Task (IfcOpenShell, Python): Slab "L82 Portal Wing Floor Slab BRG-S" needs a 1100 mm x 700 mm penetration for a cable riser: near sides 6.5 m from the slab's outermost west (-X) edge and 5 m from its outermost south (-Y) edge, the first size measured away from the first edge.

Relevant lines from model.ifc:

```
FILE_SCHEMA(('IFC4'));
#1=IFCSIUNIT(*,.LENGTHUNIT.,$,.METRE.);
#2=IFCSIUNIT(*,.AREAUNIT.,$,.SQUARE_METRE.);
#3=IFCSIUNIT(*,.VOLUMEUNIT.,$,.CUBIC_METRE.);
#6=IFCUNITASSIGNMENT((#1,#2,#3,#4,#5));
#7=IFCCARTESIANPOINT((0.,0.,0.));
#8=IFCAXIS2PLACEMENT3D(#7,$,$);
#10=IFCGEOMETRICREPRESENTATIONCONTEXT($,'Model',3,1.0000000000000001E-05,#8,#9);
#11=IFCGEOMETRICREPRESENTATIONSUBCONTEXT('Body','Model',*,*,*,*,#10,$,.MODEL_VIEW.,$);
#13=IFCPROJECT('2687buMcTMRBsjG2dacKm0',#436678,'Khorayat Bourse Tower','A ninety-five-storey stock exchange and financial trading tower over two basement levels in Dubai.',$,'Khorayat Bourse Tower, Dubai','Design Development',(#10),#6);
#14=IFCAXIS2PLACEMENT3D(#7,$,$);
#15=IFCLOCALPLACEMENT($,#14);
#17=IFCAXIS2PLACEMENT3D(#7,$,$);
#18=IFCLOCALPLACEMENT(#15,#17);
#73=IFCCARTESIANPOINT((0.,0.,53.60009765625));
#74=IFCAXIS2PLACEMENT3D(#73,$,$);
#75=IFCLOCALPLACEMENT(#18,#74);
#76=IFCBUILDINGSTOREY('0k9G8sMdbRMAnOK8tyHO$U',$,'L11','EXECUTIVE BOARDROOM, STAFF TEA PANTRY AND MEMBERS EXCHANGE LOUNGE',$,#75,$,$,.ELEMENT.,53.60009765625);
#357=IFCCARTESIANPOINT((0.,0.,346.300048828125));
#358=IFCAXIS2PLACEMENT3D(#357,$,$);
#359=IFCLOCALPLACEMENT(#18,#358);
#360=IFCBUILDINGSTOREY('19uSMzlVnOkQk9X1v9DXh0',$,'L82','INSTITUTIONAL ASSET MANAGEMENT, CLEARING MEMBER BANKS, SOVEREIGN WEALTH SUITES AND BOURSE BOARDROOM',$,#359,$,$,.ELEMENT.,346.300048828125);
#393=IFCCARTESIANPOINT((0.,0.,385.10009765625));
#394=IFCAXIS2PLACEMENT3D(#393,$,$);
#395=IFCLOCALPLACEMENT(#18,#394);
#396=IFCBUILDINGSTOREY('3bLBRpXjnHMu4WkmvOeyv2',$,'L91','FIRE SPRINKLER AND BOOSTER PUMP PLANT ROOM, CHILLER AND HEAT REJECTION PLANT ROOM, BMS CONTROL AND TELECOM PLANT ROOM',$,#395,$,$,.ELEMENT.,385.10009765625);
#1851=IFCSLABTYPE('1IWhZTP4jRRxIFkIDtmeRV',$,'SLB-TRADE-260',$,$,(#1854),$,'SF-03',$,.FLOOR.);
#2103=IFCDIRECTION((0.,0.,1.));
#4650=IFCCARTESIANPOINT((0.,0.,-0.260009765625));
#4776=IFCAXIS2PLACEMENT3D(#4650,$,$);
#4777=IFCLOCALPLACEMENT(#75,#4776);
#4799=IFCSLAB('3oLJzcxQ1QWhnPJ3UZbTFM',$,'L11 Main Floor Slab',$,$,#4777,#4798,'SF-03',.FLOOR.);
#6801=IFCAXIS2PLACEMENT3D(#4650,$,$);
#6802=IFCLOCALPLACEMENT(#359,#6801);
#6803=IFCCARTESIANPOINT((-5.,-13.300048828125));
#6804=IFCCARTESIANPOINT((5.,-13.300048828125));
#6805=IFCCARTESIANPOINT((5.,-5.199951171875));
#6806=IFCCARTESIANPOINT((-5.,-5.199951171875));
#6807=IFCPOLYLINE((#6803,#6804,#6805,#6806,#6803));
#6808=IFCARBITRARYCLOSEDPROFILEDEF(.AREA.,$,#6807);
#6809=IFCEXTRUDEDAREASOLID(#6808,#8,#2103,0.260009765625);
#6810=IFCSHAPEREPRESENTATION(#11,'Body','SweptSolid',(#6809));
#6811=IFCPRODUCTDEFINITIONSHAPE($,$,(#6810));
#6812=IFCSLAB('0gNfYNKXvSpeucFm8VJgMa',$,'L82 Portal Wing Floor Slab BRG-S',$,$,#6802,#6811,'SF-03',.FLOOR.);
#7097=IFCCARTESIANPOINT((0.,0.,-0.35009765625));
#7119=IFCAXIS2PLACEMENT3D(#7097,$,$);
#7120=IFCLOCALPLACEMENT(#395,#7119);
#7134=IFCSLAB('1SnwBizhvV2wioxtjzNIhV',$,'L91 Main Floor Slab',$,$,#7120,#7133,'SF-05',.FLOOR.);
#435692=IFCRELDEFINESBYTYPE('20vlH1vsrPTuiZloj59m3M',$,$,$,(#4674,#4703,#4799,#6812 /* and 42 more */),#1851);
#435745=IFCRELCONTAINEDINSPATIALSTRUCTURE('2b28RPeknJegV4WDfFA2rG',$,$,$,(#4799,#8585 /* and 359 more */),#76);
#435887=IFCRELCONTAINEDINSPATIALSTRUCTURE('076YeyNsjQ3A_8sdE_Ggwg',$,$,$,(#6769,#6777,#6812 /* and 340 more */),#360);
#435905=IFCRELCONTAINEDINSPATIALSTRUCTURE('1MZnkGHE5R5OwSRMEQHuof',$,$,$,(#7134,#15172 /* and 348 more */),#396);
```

```python
import numpy as np
import ifcopenshell
import ifcopenshell.api.feature
import ifcopenshell.api.geometry
import ifcopenshell.api.root
import ifcopenshell.geom
import ifcopenshell.util.placement
import ifcopenshell.util.representation
import ifcopenshell.util.shape
import ifcopenshell.util.unit

model = ifcopenshell.open("model.ifc")
unit_scale = ifcopenshell.util.unit.calculate_unit_scale(model)
settings = ifcopenshell.geom.settings()


def volume(element):
    """Net volume in cubic metres, openings subtracted."""
    shape = ifcopenshell.geom.create_shape(settings, element)
    return ifcopenshell.util.shape.get_volume(shape.geometry)


slab = model.by_id(6812)
before = volume(slab)

# Extent in the slab's own axes, in metres. The edges named are its -X and -Y sides.
slab_shape = ifcopenshell.geom.create_shape(settings, slab)
vertices = ifcopenshell.util.shape.get_vertices(slab_shape.geometry)
x_min, y_min, bottom = vertices.min(axis=0)
top = vertices[:, 2].max()

opening = ifcopenshell.api.root.create_entity(model, ifc_class="IfcOpeningElement", name="Cable riser opening", predefined_type="OPENING")
context = ifcopenshell.util.representation.get_context(model, "Model", "Body", "MODEL_VIEW")
width, depth = 1.1, 0.7
outline = [(0.0, 0.0), (width, 0.0), (width, depth), (0.0, depth), (0.0, 0.0)]
# Overshoot both faces by 50 mm so the cut is clean.
shape = ifcopenshell.api.geometry.add_slab_representation(
    model, context=context, depth=top - bottom + 0.1, polyline=outline
)
ifcopenshell.api.geometry.assign_representation(model, product=opening, representation=shape)

matrix = ifcopenshell.util.placement.get_local_placement(slab.ObjectPlacement)
matrix[:, 3] = matrix @ np.append(np.array([x_min + 6.5, y_min + 5, bottom - 0.05]) / unit_scale, 1.0)
ifcopenshell.api.geometry.edit_object_placement(model, product=opening, matrix=matrix, is_si=False)
ifcopenshell.api.feature.add_feature(model, feature=opening, element=slab)

after = volume(slab)

print(f"slab volume {before:.3f} -> {after:.3f} m3")

model.write("model_edited.ifc")
```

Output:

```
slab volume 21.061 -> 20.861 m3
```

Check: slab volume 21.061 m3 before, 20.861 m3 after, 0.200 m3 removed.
